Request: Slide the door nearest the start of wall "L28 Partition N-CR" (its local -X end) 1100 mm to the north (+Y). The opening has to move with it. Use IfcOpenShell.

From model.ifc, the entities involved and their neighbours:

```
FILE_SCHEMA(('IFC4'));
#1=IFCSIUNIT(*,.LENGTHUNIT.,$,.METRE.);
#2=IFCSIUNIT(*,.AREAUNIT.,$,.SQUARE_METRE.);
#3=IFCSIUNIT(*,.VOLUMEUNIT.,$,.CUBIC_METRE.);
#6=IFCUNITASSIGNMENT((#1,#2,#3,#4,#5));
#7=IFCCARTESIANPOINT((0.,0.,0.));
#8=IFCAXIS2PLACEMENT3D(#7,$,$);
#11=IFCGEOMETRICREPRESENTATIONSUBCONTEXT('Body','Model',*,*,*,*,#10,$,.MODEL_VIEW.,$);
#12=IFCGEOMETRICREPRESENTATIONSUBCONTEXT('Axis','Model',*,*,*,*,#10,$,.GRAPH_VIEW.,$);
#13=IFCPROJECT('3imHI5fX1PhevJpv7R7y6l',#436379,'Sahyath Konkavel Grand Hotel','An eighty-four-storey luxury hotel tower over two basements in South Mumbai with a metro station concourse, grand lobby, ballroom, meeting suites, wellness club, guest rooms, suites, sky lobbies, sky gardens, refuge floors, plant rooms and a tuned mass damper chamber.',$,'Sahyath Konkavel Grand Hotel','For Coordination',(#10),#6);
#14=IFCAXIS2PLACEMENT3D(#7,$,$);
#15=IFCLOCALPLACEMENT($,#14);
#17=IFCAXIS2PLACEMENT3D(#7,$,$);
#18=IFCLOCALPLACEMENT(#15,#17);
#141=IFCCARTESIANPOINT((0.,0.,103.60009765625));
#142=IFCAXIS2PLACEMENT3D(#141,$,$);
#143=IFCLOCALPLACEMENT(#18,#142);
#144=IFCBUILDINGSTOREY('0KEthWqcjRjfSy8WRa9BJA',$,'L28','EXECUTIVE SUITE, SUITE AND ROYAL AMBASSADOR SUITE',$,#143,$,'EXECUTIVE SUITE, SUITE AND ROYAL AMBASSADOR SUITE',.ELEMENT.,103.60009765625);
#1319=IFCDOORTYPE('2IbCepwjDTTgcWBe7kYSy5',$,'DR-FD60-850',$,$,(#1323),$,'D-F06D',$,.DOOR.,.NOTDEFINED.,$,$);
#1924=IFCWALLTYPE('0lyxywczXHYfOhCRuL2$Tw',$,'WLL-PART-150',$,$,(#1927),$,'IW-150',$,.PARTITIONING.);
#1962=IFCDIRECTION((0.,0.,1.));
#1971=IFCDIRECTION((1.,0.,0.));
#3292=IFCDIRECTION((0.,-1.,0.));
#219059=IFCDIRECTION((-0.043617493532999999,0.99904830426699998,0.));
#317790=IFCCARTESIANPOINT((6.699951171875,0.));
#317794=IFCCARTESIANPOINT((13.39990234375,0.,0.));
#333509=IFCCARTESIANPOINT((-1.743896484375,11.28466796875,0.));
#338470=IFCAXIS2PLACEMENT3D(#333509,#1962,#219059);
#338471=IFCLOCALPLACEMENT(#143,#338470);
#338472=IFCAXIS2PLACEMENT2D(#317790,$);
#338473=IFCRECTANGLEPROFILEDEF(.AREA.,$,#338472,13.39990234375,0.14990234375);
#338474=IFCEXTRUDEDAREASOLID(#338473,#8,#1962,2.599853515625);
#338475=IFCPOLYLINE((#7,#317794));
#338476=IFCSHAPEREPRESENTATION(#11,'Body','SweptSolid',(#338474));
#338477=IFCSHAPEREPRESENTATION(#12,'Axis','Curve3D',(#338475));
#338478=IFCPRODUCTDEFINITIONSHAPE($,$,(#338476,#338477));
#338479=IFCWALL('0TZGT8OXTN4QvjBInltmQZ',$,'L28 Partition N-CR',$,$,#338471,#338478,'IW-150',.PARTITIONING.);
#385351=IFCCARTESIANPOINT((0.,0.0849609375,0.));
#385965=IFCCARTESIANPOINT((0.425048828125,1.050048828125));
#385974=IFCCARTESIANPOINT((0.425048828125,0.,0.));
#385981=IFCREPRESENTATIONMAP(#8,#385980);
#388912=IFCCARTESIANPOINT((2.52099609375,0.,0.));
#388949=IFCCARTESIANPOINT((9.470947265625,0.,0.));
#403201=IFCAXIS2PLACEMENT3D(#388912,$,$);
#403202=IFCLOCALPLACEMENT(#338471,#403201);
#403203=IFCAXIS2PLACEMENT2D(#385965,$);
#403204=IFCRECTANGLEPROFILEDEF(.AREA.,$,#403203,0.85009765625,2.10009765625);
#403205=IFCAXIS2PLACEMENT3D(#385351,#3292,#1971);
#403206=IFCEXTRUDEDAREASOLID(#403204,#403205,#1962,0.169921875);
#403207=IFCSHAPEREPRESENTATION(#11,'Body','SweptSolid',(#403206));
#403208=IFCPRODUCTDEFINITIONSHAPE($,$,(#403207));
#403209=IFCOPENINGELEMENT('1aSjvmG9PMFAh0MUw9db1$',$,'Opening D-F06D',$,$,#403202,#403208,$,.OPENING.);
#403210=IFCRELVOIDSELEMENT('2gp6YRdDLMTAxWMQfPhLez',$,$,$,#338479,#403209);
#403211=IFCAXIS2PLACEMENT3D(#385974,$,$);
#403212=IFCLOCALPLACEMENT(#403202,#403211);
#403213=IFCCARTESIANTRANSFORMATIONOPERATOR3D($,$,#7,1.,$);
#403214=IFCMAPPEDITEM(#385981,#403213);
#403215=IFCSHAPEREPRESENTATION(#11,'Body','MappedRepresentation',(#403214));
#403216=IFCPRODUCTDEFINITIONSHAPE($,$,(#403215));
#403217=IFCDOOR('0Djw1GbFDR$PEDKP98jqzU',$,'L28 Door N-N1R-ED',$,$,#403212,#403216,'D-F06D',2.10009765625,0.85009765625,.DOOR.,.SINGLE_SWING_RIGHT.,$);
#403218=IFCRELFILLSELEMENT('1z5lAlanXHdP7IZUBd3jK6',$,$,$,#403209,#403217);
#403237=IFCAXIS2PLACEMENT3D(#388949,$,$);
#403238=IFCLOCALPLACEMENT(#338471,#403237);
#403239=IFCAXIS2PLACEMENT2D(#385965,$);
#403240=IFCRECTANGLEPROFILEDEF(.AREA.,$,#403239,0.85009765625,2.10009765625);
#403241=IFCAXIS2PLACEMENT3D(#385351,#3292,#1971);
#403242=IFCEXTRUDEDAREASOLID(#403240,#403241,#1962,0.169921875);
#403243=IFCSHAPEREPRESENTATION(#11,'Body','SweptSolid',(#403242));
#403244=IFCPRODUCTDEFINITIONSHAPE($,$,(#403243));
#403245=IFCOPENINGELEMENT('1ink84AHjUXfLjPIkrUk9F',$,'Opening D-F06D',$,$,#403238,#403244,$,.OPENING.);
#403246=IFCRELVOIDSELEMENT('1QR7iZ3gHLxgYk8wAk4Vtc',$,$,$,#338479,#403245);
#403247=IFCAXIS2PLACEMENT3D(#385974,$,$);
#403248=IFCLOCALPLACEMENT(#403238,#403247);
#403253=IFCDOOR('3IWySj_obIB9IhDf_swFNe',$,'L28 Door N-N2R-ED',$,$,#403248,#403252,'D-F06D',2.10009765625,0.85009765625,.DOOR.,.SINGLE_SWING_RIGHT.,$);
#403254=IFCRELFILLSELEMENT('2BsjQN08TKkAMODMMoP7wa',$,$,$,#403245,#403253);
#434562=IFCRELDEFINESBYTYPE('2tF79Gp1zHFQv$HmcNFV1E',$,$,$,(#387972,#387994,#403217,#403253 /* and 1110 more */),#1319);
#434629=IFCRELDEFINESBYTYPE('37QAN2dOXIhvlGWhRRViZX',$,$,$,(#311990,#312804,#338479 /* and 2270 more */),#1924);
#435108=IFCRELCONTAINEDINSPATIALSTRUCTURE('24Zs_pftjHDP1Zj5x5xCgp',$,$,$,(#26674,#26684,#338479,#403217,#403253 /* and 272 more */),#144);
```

```python
import ifcopenshell
import ifcopenshell.api.geometry
import ifcopenshell.util.placement

model = ifcopenshell.open("model.ifc")

door = model.by_guid("0Djw1GbFDR$PEDKP98jqzU")
opening = door.FillsVoids[0].RelatingOpeningElement
wall = opening.VoidsElements[0].RelatingBuildingElement

wall_matrix = ifcopenshell.util.placement.get_local_placement(wall.ObjectPlacement)
shift = wall_matrix[:3, 0] * 1.1
before = ifcopenshell.util.placement.get_local_placement(door.ObjectPlacement)[:3, 3].copy()

# The door is placed relative to its opening, so it follows when the opening moves.
matrix = ifcopenshell.util.placement.get_local_placement(opening.ObjectPlacement)
matrix[:3, 3] += shift
ifcopenshell.api.geometry.edit_object_placement(
    model, product=opening, matrix=matrix, is_si=False, should_transform_children=True
)

after = ifcopenshell.util.placement.get_local_placement(door.ObjectPlacement)[:3, 3]
print("door moved by", (after - before).round(3) + 0.0)

model.write("model_rev.ifc")
```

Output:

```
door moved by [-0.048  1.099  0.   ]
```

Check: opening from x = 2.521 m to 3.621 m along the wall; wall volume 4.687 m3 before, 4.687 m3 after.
